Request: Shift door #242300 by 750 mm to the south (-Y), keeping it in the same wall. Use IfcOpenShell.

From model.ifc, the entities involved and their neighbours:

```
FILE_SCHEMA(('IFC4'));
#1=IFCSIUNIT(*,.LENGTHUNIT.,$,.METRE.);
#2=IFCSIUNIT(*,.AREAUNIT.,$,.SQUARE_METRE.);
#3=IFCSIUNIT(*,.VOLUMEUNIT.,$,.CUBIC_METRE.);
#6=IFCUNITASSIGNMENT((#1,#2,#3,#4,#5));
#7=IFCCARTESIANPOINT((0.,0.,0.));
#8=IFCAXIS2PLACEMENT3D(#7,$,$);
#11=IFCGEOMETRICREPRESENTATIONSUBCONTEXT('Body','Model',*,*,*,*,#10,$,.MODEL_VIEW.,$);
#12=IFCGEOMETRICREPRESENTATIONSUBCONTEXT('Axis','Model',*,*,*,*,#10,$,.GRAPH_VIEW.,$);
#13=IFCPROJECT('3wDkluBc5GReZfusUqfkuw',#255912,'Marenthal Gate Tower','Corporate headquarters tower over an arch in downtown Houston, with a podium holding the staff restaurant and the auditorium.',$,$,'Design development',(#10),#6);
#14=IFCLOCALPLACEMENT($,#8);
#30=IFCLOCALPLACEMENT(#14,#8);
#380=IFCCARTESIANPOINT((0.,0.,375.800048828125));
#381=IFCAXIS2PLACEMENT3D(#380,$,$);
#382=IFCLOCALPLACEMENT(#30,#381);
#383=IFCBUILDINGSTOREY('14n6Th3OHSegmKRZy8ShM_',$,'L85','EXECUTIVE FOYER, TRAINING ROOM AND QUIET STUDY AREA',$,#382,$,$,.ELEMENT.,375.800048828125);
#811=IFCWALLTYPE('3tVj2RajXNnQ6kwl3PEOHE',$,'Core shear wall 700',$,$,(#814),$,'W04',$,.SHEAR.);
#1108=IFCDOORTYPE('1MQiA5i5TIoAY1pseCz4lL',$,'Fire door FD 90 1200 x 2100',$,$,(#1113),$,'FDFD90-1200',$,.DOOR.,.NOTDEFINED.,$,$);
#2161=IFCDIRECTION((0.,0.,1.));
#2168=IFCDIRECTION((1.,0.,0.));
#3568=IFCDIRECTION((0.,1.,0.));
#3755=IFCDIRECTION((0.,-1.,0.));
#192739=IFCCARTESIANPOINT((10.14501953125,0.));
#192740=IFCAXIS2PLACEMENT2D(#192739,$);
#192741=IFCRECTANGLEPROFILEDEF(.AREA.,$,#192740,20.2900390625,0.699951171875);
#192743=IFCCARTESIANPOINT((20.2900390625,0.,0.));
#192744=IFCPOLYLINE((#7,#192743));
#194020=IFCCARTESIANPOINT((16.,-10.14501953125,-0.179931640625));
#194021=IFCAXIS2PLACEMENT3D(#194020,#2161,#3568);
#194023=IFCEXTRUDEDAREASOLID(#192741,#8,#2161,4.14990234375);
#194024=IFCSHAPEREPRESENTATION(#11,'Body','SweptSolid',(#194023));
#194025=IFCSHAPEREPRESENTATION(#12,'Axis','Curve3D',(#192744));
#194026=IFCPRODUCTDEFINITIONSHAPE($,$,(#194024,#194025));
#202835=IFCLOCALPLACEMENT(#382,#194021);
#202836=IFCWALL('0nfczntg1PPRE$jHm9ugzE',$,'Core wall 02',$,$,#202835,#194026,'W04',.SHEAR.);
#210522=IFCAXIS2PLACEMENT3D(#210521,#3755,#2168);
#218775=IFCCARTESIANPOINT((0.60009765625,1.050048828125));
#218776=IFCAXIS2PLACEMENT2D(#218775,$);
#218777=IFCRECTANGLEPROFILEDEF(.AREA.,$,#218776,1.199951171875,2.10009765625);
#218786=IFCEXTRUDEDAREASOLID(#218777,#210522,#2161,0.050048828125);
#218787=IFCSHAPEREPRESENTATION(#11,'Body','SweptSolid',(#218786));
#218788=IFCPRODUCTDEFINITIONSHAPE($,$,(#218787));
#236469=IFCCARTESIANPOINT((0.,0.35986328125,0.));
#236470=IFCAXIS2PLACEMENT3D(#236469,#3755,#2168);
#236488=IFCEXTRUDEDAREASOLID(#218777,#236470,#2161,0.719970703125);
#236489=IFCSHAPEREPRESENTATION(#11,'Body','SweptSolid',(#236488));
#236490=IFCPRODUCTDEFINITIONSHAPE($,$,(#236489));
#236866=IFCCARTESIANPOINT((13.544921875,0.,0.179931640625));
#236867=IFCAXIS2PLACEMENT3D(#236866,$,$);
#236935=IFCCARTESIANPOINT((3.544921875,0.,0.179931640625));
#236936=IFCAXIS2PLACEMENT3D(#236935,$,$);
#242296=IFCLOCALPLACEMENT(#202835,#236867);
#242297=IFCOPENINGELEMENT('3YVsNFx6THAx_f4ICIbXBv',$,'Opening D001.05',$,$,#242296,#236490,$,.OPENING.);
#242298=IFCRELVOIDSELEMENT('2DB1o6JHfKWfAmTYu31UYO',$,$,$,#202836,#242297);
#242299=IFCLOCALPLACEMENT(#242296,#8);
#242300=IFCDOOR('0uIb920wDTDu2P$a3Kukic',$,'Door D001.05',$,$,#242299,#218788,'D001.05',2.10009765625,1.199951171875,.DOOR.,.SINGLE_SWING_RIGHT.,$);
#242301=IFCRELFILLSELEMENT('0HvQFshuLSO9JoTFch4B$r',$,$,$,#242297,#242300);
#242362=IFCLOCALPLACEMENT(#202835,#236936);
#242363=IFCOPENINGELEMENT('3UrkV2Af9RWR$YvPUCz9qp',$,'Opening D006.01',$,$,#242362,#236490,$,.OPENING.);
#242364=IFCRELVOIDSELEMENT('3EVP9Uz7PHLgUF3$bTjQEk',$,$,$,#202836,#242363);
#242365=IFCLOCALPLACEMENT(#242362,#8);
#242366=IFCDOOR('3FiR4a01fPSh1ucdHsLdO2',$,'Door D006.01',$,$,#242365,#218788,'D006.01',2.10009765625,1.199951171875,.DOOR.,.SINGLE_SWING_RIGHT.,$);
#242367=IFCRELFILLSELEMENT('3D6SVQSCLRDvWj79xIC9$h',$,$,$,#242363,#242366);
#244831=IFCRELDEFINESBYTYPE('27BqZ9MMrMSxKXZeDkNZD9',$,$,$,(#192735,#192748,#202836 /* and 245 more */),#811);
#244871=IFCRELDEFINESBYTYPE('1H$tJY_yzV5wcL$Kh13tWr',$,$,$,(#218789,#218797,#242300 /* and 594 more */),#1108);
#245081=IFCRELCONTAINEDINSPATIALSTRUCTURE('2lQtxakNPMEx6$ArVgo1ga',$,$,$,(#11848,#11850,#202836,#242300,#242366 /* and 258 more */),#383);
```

```python
import ifcopenshell
import ifcopenshell.api.geometry
import ifcopenshell.util.placement

model = ifcopenshell.open("model.ifc")

door = model.by_guid("0uIb920wDTDu2P$a3Kukic")
opening = door.FillsVoids[0].RelatingOpeningElement
wall = opening.VoidsElements[0].RelatingBuildingElement

wall_matrix = ifcopenshell.util.placement.get_local_placement(wall.ObjectPlacement)
shift = wall_matrix[:3, 0] * -0.75
before = ifcopenshell.util.placement.get_local_placement(door.ObjectPlacement)[:3, 3].copy()

# The door is placed relative to its opening, so it follows when the opening moves.
matrix = ifcopenshell.util.placement.get_local_placement(opening.ObjectPlacement)
matrix[:3, 3] += shift
ifcopenshell.api.geometry.edit_object_placement(
    model, product=opening, matrix=matrix, is_si=False, should_transform_children=True
)

after = ifcopenshell.util.placement.get_local_placement(door.ObjectPlacement)[:3, 3]
print("door moved by", (after - before).round(3) + 0.0)

model.write("model_updated.ifc")
```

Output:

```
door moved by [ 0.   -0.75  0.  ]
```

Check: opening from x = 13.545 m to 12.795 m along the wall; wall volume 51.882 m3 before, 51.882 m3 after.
